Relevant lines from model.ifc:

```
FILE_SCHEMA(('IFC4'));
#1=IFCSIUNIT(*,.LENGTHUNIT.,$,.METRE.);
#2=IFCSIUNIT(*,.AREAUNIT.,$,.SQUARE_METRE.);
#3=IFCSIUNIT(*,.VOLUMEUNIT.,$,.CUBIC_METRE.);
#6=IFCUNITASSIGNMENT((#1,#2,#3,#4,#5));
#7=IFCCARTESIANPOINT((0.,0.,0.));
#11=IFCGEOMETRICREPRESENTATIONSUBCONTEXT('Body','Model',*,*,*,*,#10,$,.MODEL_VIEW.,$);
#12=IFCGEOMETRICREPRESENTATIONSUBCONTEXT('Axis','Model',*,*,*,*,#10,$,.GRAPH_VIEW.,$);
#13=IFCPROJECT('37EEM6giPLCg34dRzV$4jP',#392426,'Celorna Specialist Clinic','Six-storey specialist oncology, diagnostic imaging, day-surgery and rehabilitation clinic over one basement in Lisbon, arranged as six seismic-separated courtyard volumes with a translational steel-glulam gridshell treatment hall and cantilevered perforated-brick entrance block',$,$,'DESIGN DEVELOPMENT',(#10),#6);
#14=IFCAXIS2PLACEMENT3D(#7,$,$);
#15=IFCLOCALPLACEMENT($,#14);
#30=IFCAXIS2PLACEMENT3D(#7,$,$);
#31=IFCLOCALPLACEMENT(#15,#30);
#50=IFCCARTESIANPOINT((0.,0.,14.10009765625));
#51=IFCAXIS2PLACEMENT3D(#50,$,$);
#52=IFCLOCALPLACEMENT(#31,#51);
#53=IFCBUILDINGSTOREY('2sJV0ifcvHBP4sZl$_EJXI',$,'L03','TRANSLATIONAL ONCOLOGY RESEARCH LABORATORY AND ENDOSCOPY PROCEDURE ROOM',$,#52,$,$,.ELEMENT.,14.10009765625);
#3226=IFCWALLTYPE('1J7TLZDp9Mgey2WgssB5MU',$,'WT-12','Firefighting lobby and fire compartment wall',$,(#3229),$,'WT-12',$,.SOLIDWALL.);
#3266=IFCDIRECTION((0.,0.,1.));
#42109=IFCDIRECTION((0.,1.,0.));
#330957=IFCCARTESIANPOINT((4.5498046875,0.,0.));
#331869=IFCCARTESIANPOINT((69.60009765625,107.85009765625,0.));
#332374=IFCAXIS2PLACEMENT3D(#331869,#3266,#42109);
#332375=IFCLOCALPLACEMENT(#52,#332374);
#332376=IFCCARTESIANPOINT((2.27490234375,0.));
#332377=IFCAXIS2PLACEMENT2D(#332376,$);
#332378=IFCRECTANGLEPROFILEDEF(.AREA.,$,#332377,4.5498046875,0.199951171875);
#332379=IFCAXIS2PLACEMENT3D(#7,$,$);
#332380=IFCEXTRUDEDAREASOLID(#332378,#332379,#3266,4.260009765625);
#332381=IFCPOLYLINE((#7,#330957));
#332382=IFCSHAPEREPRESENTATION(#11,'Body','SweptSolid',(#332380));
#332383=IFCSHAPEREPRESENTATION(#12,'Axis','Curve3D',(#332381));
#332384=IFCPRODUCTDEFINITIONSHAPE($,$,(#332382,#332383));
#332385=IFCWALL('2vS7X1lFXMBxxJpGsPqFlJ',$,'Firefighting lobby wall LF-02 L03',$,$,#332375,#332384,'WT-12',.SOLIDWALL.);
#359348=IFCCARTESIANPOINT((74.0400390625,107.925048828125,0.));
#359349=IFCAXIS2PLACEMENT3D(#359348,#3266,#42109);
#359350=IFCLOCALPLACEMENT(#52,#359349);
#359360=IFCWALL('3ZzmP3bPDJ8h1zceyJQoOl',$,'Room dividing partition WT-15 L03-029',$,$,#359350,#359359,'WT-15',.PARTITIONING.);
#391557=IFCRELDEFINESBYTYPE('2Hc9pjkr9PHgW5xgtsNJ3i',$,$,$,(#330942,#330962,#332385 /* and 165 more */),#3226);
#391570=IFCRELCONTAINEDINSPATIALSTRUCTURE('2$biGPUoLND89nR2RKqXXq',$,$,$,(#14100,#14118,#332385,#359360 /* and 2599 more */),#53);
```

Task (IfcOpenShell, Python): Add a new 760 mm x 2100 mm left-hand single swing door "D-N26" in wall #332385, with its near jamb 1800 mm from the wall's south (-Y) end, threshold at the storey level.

```python
import numpy as np
import ifcopenshell
import ifcopenshell.api.feature
import ifcopenshell.api.geometry
import ifcopenshell.api.root
import ifcopenshell.api.spatial
import ifcopenshell.geom
import ifcopenshell.util.element
import ifcopenshell.util.placement
import ifcopenshell.util.representation
import ifcopenshell.util.shape
import ifcopenshell.util.unit

model = ifcopenshell.open("model.ifc")
unit_scale = ifcopenshell.util.unit.calculate_unit_scale(model)
settings = ifcopenshell.geom.settings()


def volume(element):
    """Net volume in cubic metres, openings subtracted."""
    shape = ifcopenshell.geom.create_shape(settings, element)
    return ifcopenshell.util.shape.get_volume(shape.geometry)


wall = model.by_guid("2vS7X1lFXMBxxJpGsPqFlJ")
storey = ifcopenshell.util.element.get_container(wall, ifc_class="IfcBuildingStorey")
context = ifcopenshell.util.representation.get_context(model, "Model", "Body", "MODEL_VIEW")
before = volume(wall)

width, height, from_end, sill = 0.76, 2.1, 1.8, 0.0  # metres

# The wall runs along its own X axis, and the end named is its -X end.
wall_shape = ifcopenshell.geom.create_shape(settings, wall)
x, y, z = ifcopenshell.util.shape.get_vertices(wall_shape.geometry).T
start = x.min() + from_end
face, thickness = float(y.min()), float(y.max() - y.min())
wall_matrix = ifcopenshell.util.placement.get_local_placement(wall.ObjectPlacement)
level = ifcopenshell.util.placement.get_local_placement(storey.ObjectPlacement)[2, 3]


def in_wall(x, y):
    """Placement at x, y metres in the wall's axes, at sill height."""
    matrix = wall_matrix.copy()
    matrix[:, 3] = wall_matrix @ np.array([x / unit_scale, y / unit_scale, 0.0, 1.0])
    matrix[2, 3] = level + sill / unit_scale
    return matrix


# Opening: a box that overshoots both wall faces by 50 mm.
opening = ifcopenshell.api.root.create_entity(model, ifc_class="IfcOpeningElement", predefined_type="OPENING")
box = ifcopenshell.api.geometry.add_wall_representation(
    model, context=context, length=width, height=height, thickness=thickness + 0.1
)
ifcopenshell.api.geometry.assign_representation(model, product=opening, representation=box)
ifcopenshell.api.geometry.edit_object_placement(model, product=opening, matrix=in_wall(start, face - 0.05), is_si=False)
ifcopenshell.api.feature.add_feature(model, feature=opening, element=wall)

door = ifcopenshell.api.root.create_entity(model, ifc_class="IfcDoor", name="D-N26", predefined_type="DOOR")
door.OverallWidth, door.OverallHeight = width / unit_scale, height / unit_scale
door.OperationType = "SINGLE_SWING_LEFT"
body = ifcopenshell.api.geometry.add_door_representation(
    model,
    context=context,
    overall_width=door.OverallWidth,
    overall_height=door.OverallHeight,
    operation_type="SINGLE_SWING_LEFT",
    lining_properties={"LiningDepth": thickness / unit_scale, "ThresholdDepth": thickness / unit_scale},
)
ifcopenshell.api.geometry.assign_representation(model, product=door, representation=body)
ifcopenshell.api.spatial.assign_container(model, products=[door], relating_structure=storey)
ifcopenshell.api.feature.add_filling(model, opening=opening, element=door)

# The lining spans the wall, so the door starts at the wall face.
ifcopenshell.api.geometry.edit_object_placement(model, product=door, matrix=in_wall(start, face), is_si=False)

after = volume(wall)

print(f"wall volume {before:.3f} -> {after:.3f} m3")

model.write("model_v2.ifc")
```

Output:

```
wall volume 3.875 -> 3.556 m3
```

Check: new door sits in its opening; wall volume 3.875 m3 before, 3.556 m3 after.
